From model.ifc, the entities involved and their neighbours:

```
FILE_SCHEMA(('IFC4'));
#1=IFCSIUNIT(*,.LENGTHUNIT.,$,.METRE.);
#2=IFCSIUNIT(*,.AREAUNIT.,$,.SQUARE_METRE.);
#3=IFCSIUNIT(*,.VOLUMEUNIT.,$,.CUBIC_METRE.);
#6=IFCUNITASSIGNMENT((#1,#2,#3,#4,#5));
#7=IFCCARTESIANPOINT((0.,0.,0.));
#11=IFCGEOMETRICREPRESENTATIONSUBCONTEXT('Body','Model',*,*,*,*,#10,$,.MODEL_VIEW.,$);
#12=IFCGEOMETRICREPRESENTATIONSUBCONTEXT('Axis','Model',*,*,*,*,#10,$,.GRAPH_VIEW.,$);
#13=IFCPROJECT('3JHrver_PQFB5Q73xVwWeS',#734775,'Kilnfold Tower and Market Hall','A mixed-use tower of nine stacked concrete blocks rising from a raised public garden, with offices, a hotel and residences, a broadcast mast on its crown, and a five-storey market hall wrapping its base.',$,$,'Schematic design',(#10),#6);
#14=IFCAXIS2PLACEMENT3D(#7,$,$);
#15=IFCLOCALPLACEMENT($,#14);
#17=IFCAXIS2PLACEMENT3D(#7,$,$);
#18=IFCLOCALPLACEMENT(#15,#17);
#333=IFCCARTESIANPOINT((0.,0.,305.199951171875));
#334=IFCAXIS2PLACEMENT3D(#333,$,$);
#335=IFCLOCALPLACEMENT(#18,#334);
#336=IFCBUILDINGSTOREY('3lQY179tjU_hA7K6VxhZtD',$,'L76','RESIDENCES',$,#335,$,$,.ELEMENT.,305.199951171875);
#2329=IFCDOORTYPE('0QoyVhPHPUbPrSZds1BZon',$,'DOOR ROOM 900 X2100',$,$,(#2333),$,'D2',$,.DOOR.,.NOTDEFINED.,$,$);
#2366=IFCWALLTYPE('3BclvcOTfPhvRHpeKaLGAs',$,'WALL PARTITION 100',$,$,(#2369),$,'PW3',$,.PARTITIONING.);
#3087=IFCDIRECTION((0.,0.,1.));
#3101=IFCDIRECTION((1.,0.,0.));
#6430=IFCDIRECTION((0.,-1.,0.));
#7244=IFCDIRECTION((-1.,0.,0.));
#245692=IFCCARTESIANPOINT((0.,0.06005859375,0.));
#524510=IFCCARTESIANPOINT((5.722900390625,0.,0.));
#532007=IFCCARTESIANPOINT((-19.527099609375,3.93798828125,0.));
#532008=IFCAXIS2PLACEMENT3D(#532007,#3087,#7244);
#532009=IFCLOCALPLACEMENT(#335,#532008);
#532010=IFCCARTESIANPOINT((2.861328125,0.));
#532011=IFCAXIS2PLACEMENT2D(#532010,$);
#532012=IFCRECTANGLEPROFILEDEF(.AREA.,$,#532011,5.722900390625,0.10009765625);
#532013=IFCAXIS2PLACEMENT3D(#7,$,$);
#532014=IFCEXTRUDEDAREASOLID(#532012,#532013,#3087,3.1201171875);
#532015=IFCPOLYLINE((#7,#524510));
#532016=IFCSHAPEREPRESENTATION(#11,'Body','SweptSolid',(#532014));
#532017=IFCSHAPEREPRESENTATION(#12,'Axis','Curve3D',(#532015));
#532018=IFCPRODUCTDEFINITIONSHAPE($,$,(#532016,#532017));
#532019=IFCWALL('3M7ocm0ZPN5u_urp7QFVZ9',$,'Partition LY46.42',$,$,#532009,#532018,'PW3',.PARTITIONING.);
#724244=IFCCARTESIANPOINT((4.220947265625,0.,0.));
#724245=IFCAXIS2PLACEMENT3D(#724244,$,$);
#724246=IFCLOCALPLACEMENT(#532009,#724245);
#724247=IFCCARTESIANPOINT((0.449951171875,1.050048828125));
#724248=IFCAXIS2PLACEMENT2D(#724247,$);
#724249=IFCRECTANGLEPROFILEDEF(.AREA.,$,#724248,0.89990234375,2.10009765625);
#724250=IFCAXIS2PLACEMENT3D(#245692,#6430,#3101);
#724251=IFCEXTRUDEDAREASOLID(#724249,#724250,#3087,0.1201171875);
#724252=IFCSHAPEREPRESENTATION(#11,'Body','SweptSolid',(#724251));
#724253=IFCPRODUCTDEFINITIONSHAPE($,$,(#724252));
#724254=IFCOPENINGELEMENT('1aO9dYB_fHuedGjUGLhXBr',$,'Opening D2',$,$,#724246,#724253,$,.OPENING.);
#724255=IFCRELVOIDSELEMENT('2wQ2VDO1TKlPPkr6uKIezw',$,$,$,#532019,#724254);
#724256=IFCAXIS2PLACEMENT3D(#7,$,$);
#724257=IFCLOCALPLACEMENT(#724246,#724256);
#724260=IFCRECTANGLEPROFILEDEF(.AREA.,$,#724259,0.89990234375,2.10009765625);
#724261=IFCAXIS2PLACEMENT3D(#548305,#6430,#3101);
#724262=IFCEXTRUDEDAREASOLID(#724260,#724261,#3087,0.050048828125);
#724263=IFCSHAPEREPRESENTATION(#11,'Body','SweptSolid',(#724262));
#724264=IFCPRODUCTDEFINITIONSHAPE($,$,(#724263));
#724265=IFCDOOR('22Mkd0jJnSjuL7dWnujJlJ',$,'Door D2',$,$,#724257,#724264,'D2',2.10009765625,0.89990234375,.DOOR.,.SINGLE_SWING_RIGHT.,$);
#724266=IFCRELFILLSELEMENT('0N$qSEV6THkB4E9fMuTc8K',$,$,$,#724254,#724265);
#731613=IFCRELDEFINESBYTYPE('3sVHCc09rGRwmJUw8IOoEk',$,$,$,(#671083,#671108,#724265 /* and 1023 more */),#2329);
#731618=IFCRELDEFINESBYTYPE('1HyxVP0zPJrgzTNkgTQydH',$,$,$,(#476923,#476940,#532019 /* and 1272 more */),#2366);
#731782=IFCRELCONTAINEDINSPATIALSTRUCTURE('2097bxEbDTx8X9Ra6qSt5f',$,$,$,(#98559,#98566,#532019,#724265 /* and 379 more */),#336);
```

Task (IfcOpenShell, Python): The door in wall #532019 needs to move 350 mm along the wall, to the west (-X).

```python
import ifcopenshell
import ifcopenshell.api.geometry
import ifcopenshell.util.placement

model = ifcopenshell.open("model.ifc")

door = model.by_guid("22Mkd0jJnSjuL7dWnujJlJ")
opening = door.FillsVoids[0].RelatingOpeningElement
wall = opening.VoidsElements[0].RelatingBuildingElement

wall_matrix = ifcopenshell.util.placement.get_local_placement(wall.ObjectPlacement)
shift = wall_matrix[:3, 0] * 0.35
before = ifcopenshell.util.placement.get_local_placement(door.ObjectPlacement)[:3, 3].copy()

# The door is placed relative to its opening, so it follows when the opening moves.
matrix = ifcopenshell.util.placement.get_local_placement(opening.ObjectPlacement)
matrix[:3, 3] += shift
ifcopenshell.api.geometry.edit_object_placement(
    model, product=opening, matrix=matrix, is_si=False, should_transform_children=True
)

after = ifcopenshell.util.placement.get_local_placement(door.ObjectPlacement)[:3, 3]
print("door moved by", (after - before).round(3) + 0.0)

model.write("model_v2.ifc")
```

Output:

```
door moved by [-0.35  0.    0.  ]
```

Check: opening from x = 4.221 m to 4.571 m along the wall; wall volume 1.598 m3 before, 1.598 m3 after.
